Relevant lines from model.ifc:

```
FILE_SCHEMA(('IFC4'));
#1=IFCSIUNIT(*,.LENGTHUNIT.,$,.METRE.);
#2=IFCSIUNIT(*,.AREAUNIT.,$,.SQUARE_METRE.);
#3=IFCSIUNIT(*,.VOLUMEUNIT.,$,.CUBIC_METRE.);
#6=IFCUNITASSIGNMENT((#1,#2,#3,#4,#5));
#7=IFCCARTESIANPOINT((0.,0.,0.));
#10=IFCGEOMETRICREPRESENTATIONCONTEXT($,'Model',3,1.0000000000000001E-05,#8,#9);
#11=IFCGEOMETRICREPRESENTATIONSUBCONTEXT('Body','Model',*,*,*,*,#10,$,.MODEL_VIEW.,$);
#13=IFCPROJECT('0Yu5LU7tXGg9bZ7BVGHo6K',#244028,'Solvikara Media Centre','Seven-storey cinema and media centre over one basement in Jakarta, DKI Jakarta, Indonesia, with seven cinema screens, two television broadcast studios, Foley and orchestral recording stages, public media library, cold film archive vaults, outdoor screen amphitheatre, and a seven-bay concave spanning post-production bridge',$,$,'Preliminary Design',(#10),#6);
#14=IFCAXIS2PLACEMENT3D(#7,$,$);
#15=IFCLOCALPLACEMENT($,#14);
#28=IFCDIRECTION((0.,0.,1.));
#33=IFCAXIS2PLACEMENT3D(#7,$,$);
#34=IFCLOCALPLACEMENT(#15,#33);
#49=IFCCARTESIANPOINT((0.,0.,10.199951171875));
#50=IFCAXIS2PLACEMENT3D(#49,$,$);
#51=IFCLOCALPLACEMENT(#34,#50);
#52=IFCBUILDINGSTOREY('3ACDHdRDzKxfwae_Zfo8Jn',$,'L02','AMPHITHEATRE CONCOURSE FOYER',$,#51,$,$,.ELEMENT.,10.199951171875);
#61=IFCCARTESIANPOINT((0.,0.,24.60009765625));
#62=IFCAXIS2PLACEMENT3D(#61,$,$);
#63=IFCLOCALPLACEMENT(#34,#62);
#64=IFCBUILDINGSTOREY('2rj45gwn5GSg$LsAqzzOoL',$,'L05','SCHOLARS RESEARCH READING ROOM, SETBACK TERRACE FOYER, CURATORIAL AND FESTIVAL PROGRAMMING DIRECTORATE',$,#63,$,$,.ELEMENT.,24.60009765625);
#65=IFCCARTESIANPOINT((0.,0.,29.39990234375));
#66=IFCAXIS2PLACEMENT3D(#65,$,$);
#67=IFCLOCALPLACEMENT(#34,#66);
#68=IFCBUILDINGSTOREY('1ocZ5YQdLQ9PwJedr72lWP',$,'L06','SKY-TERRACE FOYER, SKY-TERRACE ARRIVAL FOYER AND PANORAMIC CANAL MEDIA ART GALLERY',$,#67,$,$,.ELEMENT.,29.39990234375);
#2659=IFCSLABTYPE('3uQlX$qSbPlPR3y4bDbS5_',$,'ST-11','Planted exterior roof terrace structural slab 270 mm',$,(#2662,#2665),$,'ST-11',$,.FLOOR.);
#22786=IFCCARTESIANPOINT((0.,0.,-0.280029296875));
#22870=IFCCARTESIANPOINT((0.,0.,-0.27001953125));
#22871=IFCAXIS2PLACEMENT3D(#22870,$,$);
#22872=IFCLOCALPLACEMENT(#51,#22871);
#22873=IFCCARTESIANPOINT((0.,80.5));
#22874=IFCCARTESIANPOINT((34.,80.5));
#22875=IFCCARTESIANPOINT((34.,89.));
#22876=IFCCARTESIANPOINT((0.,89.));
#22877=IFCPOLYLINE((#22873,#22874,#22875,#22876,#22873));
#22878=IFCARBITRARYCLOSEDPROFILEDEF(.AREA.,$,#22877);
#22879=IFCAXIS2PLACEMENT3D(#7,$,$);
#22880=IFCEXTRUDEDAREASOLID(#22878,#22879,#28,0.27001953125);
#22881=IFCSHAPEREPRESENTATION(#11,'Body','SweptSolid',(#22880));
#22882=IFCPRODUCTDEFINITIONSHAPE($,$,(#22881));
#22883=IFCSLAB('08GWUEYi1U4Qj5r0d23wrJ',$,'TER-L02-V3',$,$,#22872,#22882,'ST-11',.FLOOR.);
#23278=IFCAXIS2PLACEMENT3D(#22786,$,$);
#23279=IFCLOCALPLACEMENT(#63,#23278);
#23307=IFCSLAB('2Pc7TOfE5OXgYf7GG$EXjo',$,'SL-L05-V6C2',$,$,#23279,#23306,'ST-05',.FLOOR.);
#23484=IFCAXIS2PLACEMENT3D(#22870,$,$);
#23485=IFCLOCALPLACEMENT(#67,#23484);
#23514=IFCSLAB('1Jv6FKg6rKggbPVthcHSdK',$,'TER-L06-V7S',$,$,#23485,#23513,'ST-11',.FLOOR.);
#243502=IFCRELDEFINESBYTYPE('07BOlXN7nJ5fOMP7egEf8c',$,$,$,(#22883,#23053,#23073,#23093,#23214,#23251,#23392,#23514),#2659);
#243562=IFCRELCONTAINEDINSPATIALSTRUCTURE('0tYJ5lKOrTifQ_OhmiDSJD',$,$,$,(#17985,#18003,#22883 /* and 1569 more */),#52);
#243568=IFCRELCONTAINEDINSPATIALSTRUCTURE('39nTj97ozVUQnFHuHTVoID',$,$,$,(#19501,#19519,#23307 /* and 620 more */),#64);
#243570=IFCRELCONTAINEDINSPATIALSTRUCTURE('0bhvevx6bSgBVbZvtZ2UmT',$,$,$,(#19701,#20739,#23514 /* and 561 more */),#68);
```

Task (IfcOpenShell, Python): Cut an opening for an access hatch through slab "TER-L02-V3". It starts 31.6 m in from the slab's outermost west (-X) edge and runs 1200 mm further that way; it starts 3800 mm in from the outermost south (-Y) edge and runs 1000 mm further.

```python
import numpy as np
import ifcopenshell
import ifcopenshell.api.feature
import ifcopenshell.api.geometry
import ifcopenshell.api.root
import ifcopenshell.geom
import ifcopenshell.util.placement
import ifcopenshell.util.representation
import ifcopenshell.util.shape
import ifcopenshell.util.unit

model = ifcopenshell.open("model.ifc")
unit_scale = ifcopenshell.util.unit.calculate_unit_scale(model)
settings = ifcopenshell.geom.settings()


def volume(element):
    """Net volume in cubic metres, openings subtracted."""
    shape = ifcopenshell.geom.create_shape(settings, element)
    return ifcopenshell.util.shape.get_volume(shape.geometry)


slab = model.by_guid("08GWUEYi1U4Qj5r0d23wrJ")
before = volume(slab)

# Extent in the slab's own axes, in metres. The edges named are its -X and -Y sides.
slab_shape = ifcopenshell.geom.create_shape(settings, slab)
vertices = ifcopenshell.util.shape.get_vertices(slab_shape.geometry)
x_min, y_min, bottom = vertices.min(axis=0)
top = vertices[:, 2].max()

opening = ifcopenshell.api.root.create_entity(model, ifc_class="IfcOpeningElement", name="Access hatch opening", predefined_type="OPENING")
context = ifcopenshell.util.representation.get_context(model, "Model", "Body", "MODEL_VIEW")
width, depth = 1.2, 1
outline = [(0.0, 0.0), (width, 0.0), (width, depth), (0.0, depth), (0.0, 0.0)]
# Overshoot both faces by 50 mm so the cut is clean.
shape = ifcopenshell.api.geometry.add_slab_representation(
    model, context=context, depth=top - bottom + 0.1, polyline=outline
)
ifcopenshell.api.geometry.assign_representation(model, product=opening, representation=shape)

matrix = ifcopenshell.util.placement.get_local_placement(slab.ObjectPlacement)
matrix[:, 3] = matrix @ np.append(np.array([x_min + 31.6, y_min + 3.8, bottom - 0.05]) / unit_scale, 1.0)
ifcopenshell.api.geometry.edit_object_placement(model, product=opening, matrix=matrix, is_si=False)
ifcopenshell.api.feature.add_feature(model, feature=opening, element=slab)

after = volume(slab)

print(f"slab volume {before:.3f} -> {after:.3f} m3")

model.write("model_edited.ifc")
```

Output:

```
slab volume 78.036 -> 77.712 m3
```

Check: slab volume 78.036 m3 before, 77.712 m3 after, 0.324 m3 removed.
